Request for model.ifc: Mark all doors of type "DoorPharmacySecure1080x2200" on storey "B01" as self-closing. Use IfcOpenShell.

First a look at what the model holds.

```python
import ifcopenshell
import ifcopenshell.util.element

model = ifcopenshell.open("model.ifc")
print(model.schema)
storey = next(s for s in model.by_type("IfcBuildingStorey") if s.Name == "B01")
doors = [e for e in ifcopenshell.util.element.get_decomposition(storey) if e.is_a("IfcDoor")]
seen = {}
for e in doors:
    element_type = ifcopenshell.util.element.get_type(e)
    key = (element_type.Name if element_type != e and element_type else None, ifcopenshell.util.element.get_pset(e, "Pset_DoorCommon", "SelfClosing"))
    seen[key] = seen.get(key, 0) + 1
for (name, value), count in sorted(seen.items(), key=str):
    print(count, "x", name, "|", value)
```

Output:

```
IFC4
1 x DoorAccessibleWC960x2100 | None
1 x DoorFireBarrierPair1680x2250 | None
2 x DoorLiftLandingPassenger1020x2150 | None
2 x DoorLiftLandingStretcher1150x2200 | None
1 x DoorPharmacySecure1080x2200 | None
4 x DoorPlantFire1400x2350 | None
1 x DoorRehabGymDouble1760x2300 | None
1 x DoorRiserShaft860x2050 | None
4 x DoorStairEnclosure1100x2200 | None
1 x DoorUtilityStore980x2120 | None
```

```python
import ifcopenshell
import ifcopenshell.api.pset
import ifcopenshell.util.element

model = ifcopenshell.open("model.ifc")

storey = next(s for s in model.by_type("IfcBuildingStorey") if s.Name == "B01")
doors = [e for e in ifcopenshell.util.element.get_decomposition(storey) if e.is_a("IfcDoor")]

count = 0
for e in doors:
    element_type = ifcopenshell.util.element.get_type(e)
    if element_type in (None, e) or element_type.Name != "DoorPharmacySecure1080x2200":
        continue
    # add_pset returns the element's existing set when there is one.
    pset = ifcopenshell.api.pset.add_pset(model, product=e, name="Pset_DoorCommon")
    ifcopenshell.api.pset.edit_pset(model, pset=pset, properties={"SelfClosing": True})
    count += 1

print(count, "doors updated")

model.write("model_v2.ifc")
```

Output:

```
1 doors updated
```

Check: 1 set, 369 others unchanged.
